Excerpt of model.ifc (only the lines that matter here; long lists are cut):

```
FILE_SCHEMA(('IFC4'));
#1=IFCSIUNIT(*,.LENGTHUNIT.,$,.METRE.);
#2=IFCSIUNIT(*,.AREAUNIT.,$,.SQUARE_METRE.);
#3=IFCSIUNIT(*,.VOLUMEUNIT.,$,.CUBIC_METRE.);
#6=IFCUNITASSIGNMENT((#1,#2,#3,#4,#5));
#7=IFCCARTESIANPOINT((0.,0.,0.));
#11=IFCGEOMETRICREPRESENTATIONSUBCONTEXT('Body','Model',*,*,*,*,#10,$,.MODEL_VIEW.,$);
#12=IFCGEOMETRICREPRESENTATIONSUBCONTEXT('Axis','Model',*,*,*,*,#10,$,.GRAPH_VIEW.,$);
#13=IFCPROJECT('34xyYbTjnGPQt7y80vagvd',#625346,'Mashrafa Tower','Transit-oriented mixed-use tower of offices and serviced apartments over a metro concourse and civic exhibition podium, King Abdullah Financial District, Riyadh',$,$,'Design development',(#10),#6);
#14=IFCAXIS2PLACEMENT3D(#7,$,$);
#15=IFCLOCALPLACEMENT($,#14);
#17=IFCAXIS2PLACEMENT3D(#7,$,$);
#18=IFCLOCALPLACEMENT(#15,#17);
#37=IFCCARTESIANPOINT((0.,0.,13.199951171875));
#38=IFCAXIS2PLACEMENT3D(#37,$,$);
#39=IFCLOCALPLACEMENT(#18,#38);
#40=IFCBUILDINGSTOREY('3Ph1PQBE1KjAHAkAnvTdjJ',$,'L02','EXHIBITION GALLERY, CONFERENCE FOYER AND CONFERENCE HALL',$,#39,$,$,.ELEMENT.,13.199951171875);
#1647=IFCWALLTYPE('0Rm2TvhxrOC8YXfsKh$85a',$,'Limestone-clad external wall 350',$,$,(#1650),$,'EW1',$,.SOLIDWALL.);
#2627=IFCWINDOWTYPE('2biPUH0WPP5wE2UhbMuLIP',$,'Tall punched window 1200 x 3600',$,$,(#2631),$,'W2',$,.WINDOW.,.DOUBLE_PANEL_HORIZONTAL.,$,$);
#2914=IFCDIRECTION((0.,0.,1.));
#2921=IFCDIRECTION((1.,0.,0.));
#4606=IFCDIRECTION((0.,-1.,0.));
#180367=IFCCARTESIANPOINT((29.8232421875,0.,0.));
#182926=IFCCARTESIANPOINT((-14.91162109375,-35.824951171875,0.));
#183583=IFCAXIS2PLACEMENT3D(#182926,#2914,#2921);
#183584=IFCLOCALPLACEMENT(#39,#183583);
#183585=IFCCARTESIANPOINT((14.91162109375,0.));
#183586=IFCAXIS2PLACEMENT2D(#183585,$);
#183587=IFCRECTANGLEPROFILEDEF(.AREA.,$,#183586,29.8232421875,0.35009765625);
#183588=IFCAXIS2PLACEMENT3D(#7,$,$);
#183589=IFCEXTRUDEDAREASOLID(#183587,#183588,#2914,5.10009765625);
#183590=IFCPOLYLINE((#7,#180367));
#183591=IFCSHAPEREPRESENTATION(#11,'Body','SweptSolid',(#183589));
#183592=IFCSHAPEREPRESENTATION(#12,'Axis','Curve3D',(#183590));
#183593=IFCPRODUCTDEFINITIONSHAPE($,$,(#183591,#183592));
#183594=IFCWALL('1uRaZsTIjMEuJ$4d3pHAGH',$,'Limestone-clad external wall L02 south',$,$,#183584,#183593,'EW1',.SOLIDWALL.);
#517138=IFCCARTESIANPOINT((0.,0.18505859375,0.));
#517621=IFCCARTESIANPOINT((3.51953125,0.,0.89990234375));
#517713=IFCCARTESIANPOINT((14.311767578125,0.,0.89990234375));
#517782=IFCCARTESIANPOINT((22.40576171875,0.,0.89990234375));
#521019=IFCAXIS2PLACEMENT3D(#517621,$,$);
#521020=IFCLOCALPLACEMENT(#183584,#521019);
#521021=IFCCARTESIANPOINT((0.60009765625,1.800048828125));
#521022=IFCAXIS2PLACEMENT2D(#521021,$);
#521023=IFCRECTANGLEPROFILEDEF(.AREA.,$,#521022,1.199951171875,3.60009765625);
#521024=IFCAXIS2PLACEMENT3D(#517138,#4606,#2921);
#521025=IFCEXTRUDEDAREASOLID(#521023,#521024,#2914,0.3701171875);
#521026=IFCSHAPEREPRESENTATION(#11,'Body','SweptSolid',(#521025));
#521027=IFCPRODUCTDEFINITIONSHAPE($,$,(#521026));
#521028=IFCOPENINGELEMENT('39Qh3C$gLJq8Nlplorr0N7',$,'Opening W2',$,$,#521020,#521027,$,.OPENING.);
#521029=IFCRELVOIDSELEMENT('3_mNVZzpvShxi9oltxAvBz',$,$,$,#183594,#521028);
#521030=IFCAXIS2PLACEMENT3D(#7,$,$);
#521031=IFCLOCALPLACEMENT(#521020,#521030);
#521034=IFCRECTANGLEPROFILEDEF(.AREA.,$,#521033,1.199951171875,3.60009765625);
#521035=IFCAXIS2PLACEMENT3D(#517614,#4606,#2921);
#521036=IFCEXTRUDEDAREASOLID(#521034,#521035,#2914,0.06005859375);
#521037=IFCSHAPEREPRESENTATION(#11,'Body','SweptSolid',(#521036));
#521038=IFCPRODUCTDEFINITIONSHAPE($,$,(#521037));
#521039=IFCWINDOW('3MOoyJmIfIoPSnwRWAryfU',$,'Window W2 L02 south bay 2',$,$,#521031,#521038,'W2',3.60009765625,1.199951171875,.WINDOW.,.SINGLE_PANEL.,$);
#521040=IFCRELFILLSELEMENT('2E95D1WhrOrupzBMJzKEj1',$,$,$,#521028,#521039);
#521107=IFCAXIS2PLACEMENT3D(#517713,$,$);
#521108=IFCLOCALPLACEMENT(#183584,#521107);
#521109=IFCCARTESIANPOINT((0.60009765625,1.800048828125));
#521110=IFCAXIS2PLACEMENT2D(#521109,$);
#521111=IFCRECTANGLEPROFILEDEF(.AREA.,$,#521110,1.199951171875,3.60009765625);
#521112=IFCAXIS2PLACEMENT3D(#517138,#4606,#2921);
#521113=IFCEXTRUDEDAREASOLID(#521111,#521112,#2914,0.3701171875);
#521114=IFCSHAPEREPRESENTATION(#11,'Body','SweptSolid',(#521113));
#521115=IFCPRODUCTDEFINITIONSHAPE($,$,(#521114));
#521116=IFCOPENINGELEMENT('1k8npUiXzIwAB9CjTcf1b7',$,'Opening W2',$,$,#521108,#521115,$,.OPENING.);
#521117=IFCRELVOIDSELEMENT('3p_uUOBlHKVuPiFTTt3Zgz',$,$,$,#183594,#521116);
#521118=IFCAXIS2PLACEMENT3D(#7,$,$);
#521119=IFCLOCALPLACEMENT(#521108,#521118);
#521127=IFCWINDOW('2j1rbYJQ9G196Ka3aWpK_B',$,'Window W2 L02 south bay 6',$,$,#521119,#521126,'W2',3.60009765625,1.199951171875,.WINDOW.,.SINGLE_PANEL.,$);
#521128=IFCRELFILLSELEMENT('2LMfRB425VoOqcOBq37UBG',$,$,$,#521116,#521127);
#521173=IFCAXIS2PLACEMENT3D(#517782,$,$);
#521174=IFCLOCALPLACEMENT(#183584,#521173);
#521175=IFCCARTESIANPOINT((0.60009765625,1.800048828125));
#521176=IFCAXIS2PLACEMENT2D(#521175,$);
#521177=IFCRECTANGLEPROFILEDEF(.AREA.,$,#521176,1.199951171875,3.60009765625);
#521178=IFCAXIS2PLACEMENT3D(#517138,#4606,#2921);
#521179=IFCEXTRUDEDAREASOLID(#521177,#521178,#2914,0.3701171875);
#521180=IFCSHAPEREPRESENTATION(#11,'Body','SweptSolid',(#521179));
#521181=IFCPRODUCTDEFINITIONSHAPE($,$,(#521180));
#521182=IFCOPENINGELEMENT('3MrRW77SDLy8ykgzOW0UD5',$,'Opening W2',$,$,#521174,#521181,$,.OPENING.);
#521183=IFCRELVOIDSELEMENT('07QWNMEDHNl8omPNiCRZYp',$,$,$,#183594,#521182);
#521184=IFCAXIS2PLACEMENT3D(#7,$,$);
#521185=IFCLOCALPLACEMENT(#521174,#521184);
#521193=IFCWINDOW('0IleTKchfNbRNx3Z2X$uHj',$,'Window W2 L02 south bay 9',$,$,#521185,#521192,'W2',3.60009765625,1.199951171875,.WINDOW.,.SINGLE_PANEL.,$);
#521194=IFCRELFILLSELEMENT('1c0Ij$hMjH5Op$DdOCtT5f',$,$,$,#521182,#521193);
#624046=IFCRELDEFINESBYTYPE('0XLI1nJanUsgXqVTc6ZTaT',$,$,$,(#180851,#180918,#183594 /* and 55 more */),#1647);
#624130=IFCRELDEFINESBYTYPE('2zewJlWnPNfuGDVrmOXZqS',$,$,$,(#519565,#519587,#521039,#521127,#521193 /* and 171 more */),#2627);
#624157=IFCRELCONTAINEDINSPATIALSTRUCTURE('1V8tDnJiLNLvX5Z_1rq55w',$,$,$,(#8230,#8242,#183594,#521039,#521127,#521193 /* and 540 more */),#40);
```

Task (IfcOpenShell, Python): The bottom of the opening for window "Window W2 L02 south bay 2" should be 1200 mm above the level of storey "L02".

```python
import numpy as np
import ifcopenshell
import ifcopenshell.api.geometry
import ifcopenshell.geom
import ifcopenshell.util.element
import ifcopenshell.util.placement
import ifcopenshell.util.shape
import ifcopenshell.util.unit

model = ifcopenshell.open("model.ifc")
unit_scale = ifcopenshell.util.unit.calculate_unit_scale(model)

window = model.by_guid("3MOoyJmIfIoPSnwRWAryfU")
opening = window.FillsVoids[0].RelatingOpeningElement
storey = ifcopenshell.util.element.get_container(window, ifc_class="IfcBuildingStorey")
level = ifcopenshell.util.placement.get_local_placement(storey.ObjectPlacement)[2, 3]

# The opening's origin need not be at the sill, so measure its lowest point.
shape = ifcopenshell.geom.create_shape(ifcopenshell.geom.settings(), opening)
bottom = ifcopenshell.util.shape.get_shape_bottom_elevation(shape, shape.geometry) / unit_scale
dz = level + 1.2 / unit_scale - bottom

shift = np.array([0.0, 0.0, dz])
# The window is placed relative to its opening, so it follows when the opening moves.
matrix = ifcopenshell.util.placement.get_local_placement(opening.ObjectPlacement)
matrix[:3, 3] += shift
ifcopenshell.api.geometry.edit_object_placement(
    model, product=opening, matrix=matrix, is_si=False, should_transform_children=True
)

print(f"moved by {dz * unit_scale:+.3f} m")

model.write("model_edited.ifc")
```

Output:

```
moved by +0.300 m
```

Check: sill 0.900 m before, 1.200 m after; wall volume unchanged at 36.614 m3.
